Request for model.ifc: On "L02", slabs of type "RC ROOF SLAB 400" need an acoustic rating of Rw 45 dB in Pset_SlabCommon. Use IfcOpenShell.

First a look at what the model holds.

```python
import ifcopenshell
import ifcopenshell.util.element

model = ifcopenshell.open("model.ifc")
print(model.schema)
storey = next(s for s in model.by_type("IfcBuildingStorey") if s.Name == "L02")
slabs = [e for e in ifcopenshell.util.element.get_decomposition(storey) if e.is_a("IfcSlab")]
seen = {}
for e in slabs:
    element_type = ifcopenshell.util.element.get_type(e)
    key = (element_type.Name if element_type != e and element_type else None, ifcopenshell.util.element.get_pset(e, "Pset_SlabCommon", "AcousticRating"))
    seen[key] = seen.get(key, 0) + 1
for (name, value), count in sorted(seen.items(), key=str):
    print(count, "x", name, "|", value)
```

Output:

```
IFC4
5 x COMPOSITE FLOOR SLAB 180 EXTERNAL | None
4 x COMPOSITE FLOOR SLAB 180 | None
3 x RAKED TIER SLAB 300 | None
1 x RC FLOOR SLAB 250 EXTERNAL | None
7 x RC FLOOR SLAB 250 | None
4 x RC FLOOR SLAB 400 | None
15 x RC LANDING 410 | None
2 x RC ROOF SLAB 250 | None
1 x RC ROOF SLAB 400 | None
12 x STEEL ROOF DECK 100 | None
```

```python
import ifcopenshell
import ifcopenshell.api.pset
import ifcopenshell.util.element

model = ifcopenshell.open("model.ifc")

storey = next(s for s in model.by_type("IfcBuildingStorey") if s.Name == "L02")
slabs = [e for e in ifcopenshell.util.element.get_decomposition(storey) if e.is_a("IfcSlab")]

count = 0
for e in slabs:
    element_type = ifcopenshell.util.element.get_type(e)
    if element_type in (None, e) or element_type.Name != "RC ROOF SLAB 400":
        continue
    # add_pset returns the element's existing set when there is one.
    pset = ifcopenshell.api.pset.add_pset(model, product=e, name="Pset_SlabCommon")
    ifcopenshell.api.pset.edit_pset(model, pset=pset, properties={"AcousticRating": "Rw 45 dB"})
    count += 1

print(count, "slabs updated")

model.write("model_v2.ifc")
```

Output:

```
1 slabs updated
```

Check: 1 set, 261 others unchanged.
